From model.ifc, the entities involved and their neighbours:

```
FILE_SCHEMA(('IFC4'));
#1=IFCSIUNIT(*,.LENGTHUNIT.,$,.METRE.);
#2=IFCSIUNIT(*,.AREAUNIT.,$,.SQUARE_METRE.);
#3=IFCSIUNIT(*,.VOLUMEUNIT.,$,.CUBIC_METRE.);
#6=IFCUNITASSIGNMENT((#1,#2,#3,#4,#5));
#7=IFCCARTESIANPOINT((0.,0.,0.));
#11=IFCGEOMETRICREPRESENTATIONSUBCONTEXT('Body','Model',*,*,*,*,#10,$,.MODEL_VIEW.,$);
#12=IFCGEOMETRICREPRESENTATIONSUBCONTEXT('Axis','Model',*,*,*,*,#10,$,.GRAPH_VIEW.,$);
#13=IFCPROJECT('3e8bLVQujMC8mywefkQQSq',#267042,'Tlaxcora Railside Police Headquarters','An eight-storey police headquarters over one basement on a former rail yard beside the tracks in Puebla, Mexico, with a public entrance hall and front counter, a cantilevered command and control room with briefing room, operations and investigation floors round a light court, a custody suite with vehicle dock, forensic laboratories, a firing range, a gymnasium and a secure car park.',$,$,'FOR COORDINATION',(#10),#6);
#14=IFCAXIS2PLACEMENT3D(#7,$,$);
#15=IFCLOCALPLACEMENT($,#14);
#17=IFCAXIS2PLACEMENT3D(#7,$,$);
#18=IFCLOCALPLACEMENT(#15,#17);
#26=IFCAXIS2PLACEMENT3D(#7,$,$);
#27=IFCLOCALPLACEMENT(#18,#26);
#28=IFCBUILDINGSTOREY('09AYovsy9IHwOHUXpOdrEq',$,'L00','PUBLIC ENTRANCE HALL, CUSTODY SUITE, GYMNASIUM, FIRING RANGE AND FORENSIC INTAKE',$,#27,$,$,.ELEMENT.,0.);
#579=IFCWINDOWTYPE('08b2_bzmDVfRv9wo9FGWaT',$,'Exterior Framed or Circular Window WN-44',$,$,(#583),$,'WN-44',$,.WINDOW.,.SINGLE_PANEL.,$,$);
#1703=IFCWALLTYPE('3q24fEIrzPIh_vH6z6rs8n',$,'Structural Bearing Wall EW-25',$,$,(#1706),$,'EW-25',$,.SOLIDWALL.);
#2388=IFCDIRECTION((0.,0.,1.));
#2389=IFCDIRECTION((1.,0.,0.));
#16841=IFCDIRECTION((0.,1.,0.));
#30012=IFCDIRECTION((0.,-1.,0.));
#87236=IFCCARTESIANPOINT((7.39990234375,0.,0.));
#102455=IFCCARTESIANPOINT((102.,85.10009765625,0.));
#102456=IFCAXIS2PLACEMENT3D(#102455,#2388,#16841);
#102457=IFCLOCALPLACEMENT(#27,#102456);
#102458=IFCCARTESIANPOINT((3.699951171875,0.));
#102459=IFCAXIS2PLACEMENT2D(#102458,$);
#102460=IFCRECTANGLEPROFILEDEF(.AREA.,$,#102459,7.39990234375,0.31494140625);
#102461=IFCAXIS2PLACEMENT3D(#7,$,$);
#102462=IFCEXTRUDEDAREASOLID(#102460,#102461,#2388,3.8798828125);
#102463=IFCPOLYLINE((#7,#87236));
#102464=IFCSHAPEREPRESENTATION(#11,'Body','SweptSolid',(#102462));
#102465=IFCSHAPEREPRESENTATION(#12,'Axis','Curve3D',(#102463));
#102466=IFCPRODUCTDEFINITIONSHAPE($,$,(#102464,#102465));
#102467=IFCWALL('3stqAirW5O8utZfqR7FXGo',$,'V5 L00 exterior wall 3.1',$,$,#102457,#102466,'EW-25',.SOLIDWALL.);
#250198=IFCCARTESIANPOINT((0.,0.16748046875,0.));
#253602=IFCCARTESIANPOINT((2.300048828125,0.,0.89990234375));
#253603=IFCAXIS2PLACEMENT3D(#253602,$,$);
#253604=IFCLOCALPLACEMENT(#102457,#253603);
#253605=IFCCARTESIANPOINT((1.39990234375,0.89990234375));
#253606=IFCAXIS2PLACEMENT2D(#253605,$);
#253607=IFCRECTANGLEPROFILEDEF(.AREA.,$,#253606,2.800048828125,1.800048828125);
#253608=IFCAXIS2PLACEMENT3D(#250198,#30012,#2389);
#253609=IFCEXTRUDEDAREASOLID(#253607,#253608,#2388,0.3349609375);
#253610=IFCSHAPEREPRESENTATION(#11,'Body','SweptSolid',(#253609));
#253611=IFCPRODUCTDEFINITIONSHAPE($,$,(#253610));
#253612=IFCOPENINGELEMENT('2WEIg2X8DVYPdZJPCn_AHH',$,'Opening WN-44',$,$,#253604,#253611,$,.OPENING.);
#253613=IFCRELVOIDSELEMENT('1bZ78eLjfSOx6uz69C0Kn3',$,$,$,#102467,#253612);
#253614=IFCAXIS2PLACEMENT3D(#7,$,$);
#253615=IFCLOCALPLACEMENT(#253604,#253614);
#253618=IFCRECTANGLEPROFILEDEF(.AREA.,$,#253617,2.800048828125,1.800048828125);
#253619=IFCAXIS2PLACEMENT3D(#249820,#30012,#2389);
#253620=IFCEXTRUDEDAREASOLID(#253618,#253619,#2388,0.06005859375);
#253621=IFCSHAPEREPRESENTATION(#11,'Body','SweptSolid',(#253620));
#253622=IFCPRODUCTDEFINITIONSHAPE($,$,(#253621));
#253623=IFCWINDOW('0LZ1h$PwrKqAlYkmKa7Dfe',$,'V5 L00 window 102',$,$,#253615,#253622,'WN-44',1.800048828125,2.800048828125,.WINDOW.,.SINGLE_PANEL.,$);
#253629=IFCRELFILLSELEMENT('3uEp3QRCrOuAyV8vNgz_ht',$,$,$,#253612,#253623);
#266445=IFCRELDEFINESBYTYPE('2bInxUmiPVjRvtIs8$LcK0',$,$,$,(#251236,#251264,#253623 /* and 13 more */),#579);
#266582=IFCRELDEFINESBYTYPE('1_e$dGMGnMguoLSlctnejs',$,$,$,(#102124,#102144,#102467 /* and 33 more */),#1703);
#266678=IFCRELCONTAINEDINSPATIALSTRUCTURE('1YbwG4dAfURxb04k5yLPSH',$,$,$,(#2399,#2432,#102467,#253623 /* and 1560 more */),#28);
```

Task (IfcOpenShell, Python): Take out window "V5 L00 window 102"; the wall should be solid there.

```python
import ifcopenshell
import ifcopenshell.api.feature
import ifcopenshell.api.root
import ifcopenshell.geom
import ifcopenshell.util.shape

model = ifcopenshell.open("model.ifc")
settings = ifcopenshell.geom.settings()


def volume(element):
    """Net volume in cubic metres, openings subtracted."""
    shape = ifcopenshell.geom.create_shape(settings, element)
    return ifcopenshell.util.shape.get_volume(shape.geometry)


window = model.by_id(253623)
opening = window.FillsVoids[0].RelatingOpeningElement
wall = opening.VoidsElements[0].RelatingBuildingElement
before = volume(wall)

ifcopenshell.api.root.remove_product(model, product=window)
ifcopenshell.api.feature.remove_feature(model, feature=opening)

after = volume(wall)

print(f"wall volume {before:.3f} -> {after:.3f} m3")

model.write("model_updated.ifc")
```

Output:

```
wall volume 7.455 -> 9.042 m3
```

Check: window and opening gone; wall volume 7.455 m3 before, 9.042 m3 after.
